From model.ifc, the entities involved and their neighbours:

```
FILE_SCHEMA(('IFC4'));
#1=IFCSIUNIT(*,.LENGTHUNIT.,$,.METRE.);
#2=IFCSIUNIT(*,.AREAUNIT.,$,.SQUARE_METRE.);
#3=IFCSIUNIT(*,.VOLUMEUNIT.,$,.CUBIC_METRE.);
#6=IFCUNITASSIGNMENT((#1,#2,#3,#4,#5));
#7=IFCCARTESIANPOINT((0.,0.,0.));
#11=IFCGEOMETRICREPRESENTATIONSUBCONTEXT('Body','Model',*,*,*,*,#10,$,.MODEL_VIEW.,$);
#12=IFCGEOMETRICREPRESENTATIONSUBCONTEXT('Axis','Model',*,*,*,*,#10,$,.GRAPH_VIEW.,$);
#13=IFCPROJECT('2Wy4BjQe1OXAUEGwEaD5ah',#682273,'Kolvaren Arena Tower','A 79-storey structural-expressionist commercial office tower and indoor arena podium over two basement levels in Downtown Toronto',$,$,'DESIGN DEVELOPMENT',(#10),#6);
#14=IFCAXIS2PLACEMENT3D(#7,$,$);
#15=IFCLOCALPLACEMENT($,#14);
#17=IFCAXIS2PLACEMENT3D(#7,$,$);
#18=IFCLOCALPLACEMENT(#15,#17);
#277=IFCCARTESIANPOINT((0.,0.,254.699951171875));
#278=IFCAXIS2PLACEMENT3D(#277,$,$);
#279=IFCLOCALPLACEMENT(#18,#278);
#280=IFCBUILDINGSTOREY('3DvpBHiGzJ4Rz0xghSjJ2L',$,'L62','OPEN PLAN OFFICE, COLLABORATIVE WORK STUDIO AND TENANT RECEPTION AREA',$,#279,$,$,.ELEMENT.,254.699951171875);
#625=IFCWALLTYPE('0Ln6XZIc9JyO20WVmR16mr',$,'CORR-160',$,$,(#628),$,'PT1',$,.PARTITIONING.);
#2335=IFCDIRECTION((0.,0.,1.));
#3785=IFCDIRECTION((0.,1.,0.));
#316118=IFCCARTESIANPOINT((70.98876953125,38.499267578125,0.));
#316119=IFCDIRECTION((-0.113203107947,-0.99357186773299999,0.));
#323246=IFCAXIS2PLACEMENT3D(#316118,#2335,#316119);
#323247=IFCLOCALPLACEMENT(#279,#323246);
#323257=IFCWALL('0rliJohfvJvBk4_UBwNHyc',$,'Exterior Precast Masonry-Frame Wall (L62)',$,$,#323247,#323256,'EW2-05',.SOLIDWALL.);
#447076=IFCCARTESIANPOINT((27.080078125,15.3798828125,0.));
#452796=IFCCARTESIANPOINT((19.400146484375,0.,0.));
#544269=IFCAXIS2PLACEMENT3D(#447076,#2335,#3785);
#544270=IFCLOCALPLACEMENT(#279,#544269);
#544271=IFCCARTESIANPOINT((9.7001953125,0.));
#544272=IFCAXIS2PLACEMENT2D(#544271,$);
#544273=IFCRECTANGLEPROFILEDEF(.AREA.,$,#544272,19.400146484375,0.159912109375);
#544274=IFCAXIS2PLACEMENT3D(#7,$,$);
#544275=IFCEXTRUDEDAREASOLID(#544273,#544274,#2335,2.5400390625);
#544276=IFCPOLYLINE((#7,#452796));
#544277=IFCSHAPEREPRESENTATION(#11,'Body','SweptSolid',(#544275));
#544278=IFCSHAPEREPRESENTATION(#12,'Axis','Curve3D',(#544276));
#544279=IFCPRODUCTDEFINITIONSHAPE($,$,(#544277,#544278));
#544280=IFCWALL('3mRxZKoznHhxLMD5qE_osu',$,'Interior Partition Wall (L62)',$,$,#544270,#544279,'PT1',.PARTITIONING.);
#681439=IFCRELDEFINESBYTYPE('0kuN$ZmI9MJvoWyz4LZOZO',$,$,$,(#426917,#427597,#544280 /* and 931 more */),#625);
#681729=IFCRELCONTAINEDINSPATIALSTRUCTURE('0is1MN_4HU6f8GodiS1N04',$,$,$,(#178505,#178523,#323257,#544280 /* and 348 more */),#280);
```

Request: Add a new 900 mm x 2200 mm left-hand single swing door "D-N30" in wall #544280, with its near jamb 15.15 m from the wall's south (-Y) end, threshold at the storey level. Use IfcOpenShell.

```python
import numpy as np
import ifcopenshell
import ifcopenshell.api.feature
import ifcopenshell.api.geometry
import ifcopenshell.api.root
import ifcopenshell.api.spatial
import ifcopenshell.geom
import ifcopenshell.util.element
import ifcopenshell.util.placement
import ifcopenshell.util.representation
import ifcopenshell.util.shape
import ifcopenshell.util.unit

model = ifcopenshell.open("model.ifc")
unit_scale = ifcopenshell.util.unit.calculate_unit_scale(model)
settings = ifcopenshell.geom.settings()


def volume(element):
    """Net volume in cubic metres, openings subtracted."""
    shape = ifcopenshell.geom.create_shape(settings, element)
    return ifcopenshell.util.shape.get_volume(shape.geometry)


wall = model.by_guid("3mRxZKoznHhxLMD5qE_osu")
storey = ifcopenshell.util.element.get_container(wall, ifc_class="IfcBuildingStorey")
context = ifcopenshell.util.representation.get_context(model, "Model", "Body", "MODEL_VIEW")
before = volume(wall)

width, height, from_end, sill = 0.9, 2.2, 15.15, 0.0  # metres

# The wall runs along its own X axis, and the end named is its -X end.
wall_shape = ifcopenshell.geom.create_shape(settings, wall)
x, y, z = ifcopenshell.util.shape.get_vertices(wall_shape.geometry).T
start = x.min() + from_end
face, thickness = float(y.min()), float(y.max() - y.min())
wall_matrix = ifcopenshell.util.placement.get_local_placement(wall.ObjectPlacement)
level = ifcopenshell.util.placement.get_local_placement(storey.ObjectPlacement)[2, 3]


def in_wall(x, y):
    """Placement at x, y metres in the wall's axes, at sill height."""
    matrix = wall_matrix.copy()
    matrix[:, 3] = wall_matrix @ np.array([x / unit_scale, y / unit_scale, 0.0, 1.0])
    matrix[2, 3] = level + sill / unit_scale
    return matrix


# Opening: a box that overshoots both wall faces by 50 mm.
opening = ifcopenshell.api.root.create_entity(model, ifc_class="IfcOpeningElement", predefined_type="OPENING")
box = ifcopenshell.api.geometry.add_wall_representation(
    model, context=context, length=width, height=height, thickness=thickness + 0.1
)
ifcopenshell.api.geometry.assign_representation(model, product=opening, representation=box)
ifcopenshell.api.geometry.edit_object_placement(model, product=opening, matrix=in_wall(start, face - 0.05), is_si=False)
ifcopenshell.api.feature.add_feature(model, feature=opening, element=wall)

door = ifcopenshell.api.root.create_entity(model, ifc_class="IfcDoor", name="D-N30", predefined_type="DOOR")
door.OverallWidth, door.OverallHeight = width / unit_scale, height / unit_scale
door.OperationType = "SINGLE_SWING_LEFT"
body = ifcopenshell.api.geometry.add_door_representation(
    model,
    context=context,
    overall_width=door.OverallWidth,
    overall_height=door.OverallHeight,
    operation_type="SINGLE_SWING_LEFT",
    lining_properties={"LiningDepth": thickness / unit_scale, "ThresholdDepth": thickness / unit_scale},
)
ifcopenshell.api.geometry.assign_representation(model, product=door, representation=body)
ifcopenshell.api.spatial.assign_container(model, products=[door], relating_structure=storey)
ifcopenshell.api.feature.add_filling(model, opening=opening, element=door)

# The lining spans the wall, so the door starts at the wall face.
ifcopenshell.api.geometry.edit_object_placement(model, product=door, matrix=in_wall(start, face), is_si=False)

after = volume(wall)

print(f"wall volume {before:.3f} -> {after:.3f} m3")

model.write("model-out.ifc")
```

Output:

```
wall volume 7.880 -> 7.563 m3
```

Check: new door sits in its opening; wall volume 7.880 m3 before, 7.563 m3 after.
